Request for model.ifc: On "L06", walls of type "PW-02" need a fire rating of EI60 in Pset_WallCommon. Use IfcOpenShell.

First a look at what the model holds.

```python
import ifcopenshell
import ifcopenshell.util.element

model = ifcopenshell.open("model.ifc")
print(model.schema)
storey = next(s for s in model.by_type("IfcBuildingStorey") if s.Name == "L06")
walls = [e for e in ifcopenshell.util.element.get_decomposition(storey) if e.is_a("IfcWall")]
seen = {}
for e in walls:
    element_type = ifcopenshell.util.element.get_type(e)
    key = (element_type.Name if element_type != e and element_type else None, ifcopenshell.util.element.get_pset(e, "Pset_WallCommon", "FireRating"))
    seen[key] = seen.get(key, 0) + 1
for (name, value), count in sorted(seen.items(), key=str):
    print(count, "x", name, "|", value)
```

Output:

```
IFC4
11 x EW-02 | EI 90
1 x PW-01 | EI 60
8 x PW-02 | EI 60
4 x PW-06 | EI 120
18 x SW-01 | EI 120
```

```python
import ifcopenshell
import ifcopenshell.api.pset
import ifcopenshell.util.element

model = ifcopenshell.open("model.ifc")

storey = next(s for s in model.by_type("IfcBuildingStorey") if s.Name == "L06")
walls = [e for e in ifcopenshell.util.element.get_decomposition(storey) if e.is_a("IfcWall")]

count = 0
for e in walls:
    element_type = ifcopenshell.util.element.get_type(e)
    if element_type in (None, e) or element_type.Name != "PW-02":
        continue
    # add_pset returns the element's existing set when there is one.
    pset = ifcopenshell.api.pset.add_pset(model, product=e, name="Pset_WallCommon")
    ifcopenshell.api.pset.edit_pset(model, pset=pset, properties={"FireRating": "EI60"})
    count += 1

print(count, "walls updated")

model.write("model_edited.ifc")
```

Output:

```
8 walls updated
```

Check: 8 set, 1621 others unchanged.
